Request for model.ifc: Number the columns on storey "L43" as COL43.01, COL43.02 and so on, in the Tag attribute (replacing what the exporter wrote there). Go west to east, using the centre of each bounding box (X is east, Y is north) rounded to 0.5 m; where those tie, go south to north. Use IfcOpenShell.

First a look at what the model holds.

```python
import ifcopenshell
import ifcopenshell.util.element
import ifcopenshell.util.placement

model = ifcopenshell.open("model.ifc")
print(model.schema)
storey = next(s for s in model.by_type("IfcBuildingStorey") if s.Name == "L43")
columns = [e for e in ifcopenshell.util.element.get_decomposition(storey) if e.is_a("IfcColumn")]
for e in sorted(columns, key=lambda e: e.id()):
    origin = ifcopenshell.util.placement.get_local_placement(e.ObjectPlacement)[:3, 3]
    print(e.id(), e.Tag, e.Name, origin.round(2) + 0.0, sep=" | ")
```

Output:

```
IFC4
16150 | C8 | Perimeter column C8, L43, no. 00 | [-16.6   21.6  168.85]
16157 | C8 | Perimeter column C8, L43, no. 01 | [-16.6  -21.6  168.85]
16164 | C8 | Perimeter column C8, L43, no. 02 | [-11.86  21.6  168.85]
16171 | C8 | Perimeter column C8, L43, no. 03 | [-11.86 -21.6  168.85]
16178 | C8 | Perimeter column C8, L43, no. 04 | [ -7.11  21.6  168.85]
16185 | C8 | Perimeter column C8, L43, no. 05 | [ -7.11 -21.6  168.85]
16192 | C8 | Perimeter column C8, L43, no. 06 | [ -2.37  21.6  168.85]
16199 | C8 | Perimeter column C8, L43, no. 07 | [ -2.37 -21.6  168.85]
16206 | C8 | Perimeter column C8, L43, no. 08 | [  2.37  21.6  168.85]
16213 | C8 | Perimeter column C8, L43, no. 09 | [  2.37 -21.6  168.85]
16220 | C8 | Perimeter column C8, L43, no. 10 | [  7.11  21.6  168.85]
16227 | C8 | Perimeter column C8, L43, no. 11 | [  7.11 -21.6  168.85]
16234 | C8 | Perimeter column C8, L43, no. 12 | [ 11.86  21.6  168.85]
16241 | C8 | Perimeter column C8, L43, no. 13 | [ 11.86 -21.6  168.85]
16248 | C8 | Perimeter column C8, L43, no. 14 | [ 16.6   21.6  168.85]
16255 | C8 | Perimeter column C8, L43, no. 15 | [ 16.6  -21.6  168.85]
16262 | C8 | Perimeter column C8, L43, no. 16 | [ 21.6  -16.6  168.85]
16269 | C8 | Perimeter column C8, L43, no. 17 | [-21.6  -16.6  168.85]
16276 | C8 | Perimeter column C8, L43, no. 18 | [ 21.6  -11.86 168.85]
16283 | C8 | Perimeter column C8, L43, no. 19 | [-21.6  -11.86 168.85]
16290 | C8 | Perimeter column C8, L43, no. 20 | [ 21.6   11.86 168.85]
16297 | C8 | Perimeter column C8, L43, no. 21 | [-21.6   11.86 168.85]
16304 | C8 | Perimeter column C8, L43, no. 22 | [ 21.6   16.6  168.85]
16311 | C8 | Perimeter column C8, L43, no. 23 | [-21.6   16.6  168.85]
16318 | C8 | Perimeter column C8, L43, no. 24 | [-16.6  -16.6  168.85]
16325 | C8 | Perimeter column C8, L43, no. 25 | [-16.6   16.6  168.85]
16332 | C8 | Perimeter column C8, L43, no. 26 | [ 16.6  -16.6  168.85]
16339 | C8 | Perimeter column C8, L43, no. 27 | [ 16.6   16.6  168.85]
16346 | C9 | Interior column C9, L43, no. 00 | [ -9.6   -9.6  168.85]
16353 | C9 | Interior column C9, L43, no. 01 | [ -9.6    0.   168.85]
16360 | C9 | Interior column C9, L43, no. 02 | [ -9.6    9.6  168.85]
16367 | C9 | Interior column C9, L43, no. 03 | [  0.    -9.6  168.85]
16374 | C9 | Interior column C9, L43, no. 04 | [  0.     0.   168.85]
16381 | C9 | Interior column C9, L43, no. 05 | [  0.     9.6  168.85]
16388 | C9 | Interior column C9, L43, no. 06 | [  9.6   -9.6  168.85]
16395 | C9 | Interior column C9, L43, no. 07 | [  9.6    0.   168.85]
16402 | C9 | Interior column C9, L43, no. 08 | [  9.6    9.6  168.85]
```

```python
import ifcopenshell
import ifcopenshell.geom
import ifcopenshell.util.element
import ifcopenshell.util.shape

model = ifcopenshell.open("model.ifc")
settings = ifcopenshell.geom.settings()
settings.set("use-world-coords", True)


def centre(element):
    shape = ifcopenshell.geom.create_shape(settings, element)
    return ifcopenshell.util.shape.get_bbox_centroid(shape.geometry)


storey = next(s for s in model.by_type("IfcBuildingStorey") if s.Name == "L43")
columns = [e for e in ifcopenshell.util.element.get_decomposition(storey) if e.is_a("IfcColumn")]

# Insertion points can sit at a corner or the storey origin, so sort by the geometry (in metres).
centres = {e: centre(e) for e in columns}
columns.sort(key=lambda e: (round(centres[e][0] / 0.5), centres[e][1]))

for i, e in enumerate(columns, start=1):
    number = f"COL43.{i:02d}"
    e.Tag = number
    print(e.id(), number)

model.write("model_rev.ifc")
```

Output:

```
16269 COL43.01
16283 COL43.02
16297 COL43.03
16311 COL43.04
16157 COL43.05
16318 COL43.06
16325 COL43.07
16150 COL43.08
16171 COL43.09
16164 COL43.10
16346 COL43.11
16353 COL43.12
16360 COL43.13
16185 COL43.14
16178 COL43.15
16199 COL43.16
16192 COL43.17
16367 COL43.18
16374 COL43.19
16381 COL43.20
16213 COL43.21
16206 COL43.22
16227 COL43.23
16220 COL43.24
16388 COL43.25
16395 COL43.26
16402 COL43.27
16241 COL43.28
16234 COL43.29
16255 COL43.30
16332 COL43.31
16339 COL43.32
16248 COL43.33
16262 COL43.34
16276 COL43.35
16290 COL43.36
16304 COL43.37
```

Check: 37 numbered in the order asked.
